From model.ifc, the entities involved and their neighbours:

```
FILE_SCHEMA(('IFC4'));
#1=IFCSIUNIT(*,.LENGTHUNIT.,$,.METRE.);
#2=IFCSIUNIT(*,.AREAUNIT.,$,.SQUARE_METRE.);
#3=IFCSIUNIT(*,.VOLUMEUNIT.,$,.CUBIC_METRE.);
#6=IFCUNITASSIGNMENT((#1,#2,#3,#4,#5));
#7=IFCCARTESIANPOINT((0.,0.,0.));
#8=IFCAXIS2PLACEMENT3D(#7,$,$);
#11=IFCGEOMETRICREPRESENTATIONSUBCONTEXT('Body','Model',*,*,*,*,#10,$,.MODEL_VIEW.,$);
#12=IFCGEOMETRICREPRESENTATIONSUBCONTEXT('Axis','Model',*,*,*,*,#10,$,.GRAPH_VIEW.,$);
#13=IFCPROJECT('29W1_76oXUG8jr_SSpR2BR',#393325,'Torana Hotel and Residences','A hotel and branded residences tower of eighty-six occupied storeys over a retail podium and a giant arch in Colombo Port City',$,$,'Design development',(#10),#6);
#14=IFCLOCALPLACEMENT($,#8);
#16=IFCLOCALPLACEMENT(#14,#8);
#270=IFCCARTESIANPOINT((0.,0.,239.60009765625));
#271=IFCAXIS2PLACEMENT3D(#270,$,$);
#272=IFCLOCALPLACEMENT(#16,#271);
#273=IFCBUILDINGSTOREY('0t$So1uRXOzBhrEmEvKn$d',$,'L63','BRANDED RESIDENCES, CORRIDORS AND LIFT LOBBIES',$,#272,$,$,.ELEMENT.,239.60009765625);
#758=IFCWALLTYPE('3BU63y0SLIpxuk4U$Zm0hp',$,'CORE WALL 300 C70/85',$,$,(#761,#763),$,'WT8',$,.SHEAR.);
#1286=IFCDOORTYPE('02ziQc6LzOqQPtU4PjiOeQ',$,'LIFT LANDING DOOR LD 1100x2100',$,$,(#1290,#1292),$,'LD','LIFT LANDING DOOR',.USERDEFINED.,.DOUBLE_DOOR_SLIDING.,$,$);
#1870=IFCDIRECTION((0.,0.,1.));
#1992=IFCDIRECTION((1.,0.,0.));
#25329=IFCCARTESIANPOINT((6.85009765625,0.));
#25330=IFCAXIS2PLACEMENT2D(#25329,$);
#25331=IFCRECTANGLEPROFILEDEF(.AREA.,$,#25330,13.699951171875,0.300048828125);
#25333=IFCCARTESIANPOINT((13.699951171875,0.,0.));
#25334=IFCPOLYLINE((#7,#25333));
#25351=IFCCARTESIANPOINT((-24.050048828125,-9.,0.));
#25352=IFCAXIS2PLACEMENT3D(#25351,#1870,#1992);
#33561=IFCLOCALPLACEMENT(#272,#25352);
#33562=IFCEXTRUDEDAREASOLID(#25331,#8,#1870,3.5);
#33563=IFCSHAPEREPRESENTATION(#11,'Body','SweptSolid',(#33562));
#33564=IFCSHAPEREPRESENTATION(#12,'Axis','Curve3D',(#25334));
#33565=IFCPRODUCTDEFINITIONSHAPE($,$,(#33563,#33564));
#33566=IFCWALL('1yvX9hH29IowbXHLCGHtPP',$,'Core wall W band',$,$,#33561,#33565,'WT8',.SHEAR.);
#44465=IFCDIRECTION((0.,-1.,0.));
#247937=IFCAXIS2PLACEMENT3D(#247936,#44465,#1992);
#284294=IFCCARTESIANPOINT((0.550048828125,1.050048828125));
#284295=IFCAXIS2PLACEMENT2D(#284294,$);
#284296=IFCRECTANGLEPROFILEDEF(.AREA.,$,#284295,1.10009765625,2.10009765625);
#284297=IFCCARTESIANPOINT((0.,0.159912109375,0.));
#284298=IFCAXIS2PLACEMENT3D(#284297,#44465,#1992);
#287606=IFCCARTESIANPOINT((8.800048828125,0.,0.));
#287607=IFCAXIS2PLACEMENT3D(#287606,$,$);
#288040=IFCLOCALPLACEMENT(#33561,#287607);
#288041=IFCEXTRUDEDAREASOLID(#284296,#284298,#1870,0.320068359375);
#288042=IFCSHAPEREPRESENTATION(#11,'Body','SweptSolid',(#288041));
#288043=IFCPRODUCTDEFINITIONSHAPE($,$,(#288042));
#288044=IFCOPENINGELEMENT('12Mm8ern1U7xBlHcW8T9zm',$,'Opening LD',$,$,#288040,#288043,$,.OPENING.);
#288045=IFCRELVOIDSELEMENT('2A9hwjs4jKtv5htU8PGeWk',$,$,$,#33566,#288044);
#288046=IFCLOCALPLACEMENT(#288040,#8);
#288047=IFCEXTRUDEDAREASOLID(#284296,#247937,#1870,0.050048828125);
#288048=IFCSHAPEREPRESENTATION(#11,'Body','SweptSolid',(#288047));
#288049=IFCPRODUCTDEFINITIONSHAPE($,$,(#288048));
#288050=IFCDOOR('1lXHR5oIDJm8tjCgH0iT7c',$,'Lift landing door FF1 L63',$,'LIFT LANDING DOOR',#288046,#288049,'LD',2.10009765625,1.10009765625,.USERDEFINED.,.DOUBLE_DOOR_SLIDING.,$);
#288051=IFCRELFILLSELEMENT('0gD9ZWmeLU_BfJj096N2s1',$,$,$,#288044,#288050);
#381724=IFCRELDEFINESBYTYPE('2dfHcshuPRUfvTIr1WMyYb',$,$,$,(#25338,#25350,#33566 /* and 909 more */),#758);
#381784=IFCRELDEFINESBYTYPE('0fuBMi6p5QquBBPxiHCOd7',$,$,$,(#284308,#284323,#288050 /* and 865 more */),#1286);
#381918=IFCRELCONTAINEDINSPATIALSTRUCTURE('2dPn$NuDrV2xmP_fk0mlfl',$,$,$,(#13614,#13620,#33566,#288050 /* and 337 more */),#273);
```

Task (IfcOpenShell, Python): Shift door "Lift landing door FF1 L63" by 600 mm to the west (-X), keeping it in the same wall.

```python
import ifcopenshell
import ifcopenshell.api.geometry
import ifcopenshell.util.placement
import ifcopenshell.util.unit

model = ifcopenshell.open("model.ifc")
unit_scale = ifcopenshell.util.unit.calculate_unit_scale(model)

door = model.by_id(288050)
opening = door.FillsVoids[0].RelatingOpeningElement
wall = opening.VoidsElements[0].RelatingBuildingElement

wall_matrix = ifcopenshell.util.placement.get_local_placement(wall.ObjectPlacement)
shift = wall_matrix[:3, 0] * -0.6 / unit_scale
before = ifcopenshell.util.placement.get_local_placement(door.ObjectPlacement)[:3, 3].copy()

# The door is placed relative to its opening, so it follows when the opening moves.
matrix = ifcopenshell.util.placement.get_local_placement(opening.ObjectPlacement)
matrix[:3, 3] += shift
ifcopenshell.api.geometry.edit_object_placement(
    model, product=opening, matrix=matrix, is_si=False, should_transform_children=True
)

after = ifcopenshell.util.placement.get_local_placement(door.ObjectPlacement)[:3, 3]
print("door moved by", (after - before).round(3) + 0.0)

model.write("model_rev.ifc")
```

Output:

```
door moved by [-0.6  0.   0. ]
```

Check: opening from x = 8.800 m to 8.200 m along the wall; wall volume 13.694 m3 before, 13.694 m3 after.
